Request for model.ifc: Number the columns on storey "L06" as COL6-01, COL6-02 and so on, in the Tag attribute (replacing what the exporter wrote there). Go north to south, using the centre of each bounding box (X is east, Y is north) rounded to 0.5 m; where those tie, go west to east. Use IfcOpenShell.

First a look at what the model holds.

```python
import ifcopenshell
import ifcopenshell.util.element
import ifcopenshell.util.placement

model = ifcopenshell.open("model.ifc")
print(model.schema)
storey = next(s for s in model.by_type("IfcBuildingStorey") if s.Name == "L06")
columns = [e for e in ifcopenshell.util.element.get_decomposition(storey) if e.is_a("IfcColumn")]
for e in sorted(columns, key=lambda e: e.id()):
    origin = ifcopenshell.util.placement.get_local_placement(e.ObjectPlacement)[:3, 3]
    print(e.id(), e.Tag, e.Name, origin.round(2) + 0.0, sep=" | ")
```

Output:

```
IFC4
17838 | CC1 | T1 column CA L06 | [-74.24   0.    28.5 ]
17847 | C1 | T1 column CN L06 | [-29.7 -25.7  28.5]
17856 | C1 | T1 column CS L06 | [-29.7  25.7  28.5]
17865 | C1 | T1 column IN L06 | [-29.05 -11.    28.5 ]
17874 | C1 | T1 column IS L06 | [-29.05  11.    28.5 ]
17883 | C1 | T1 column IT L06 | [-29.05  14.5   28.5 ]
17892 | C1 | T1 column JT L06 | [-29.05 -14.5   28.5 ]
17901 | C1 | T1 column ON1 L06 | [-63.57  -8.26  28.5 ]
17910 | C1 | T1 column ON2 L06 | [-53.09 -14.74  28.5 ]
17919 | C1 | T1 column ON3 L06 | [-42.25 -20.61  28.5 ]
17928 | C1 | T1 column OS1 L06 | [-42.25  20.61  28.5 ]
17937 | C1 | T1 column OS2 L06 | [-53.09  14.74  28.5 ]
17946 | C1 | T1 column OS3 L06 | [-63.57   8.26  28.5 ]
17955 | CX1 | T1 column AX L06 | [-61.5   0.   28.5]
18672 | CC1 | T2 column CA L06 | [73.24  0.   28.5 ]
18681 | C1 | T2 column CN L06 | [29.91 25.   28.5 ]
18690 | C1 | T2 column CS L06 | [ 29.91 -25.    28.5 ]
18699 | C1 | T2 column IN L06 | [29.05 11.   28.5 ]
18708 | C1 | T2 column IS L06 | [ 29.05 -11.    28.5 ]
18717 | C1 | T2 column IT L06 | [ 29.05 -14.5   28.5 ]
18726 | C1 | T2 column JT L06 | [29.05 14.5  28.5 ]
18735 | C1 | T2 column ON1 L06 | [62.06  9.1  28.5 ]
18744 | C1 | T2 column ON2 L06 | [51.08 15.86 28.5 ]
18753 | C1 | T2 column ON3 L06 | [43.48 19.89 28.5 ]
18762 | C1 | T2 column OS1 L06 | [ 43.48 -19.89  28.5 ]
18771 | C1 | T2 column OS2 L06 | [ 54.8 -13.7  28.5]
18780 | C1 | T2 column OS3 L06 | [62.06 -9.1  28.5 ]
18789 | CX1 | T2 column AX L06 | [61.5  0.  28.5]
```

```python
import ifcopenshell
import ifcopenshell.geom
import ifcopenshell.util.element
import ifcopenshell.util.shape

model = ifcopenshell.open("model.ifc")
settings = ifcopenshell.geom.settings()
settings.set("use-world-coords", True)


def centre(element):
    shape = ifcopenshell.geom.create_shape(settings, element)
    return ifcopenshell.util.shape.get_bbox_centroid(shape.geometry)


storey = next(s for s in model.by_type("IfcBuildingStorey") if s.Name == "L06")
columns = [e for e in ifcopenshell.util.element.get_decomposition(storey) if e.is_a("IfcColumn")]

# Insertion points can sit at a corner or the storey origin, so sort by the geometry (in metres).
centres = {e: centre(e) for e in columns}
columns.sort(key=lambda e: (-round(centres[e][1] / 0.5), centres[e][0]))

for i, e in enumerate(columns, start=1):
    number = f"COL6-{i:02d}"
    e.Tag = number
    print(e.id(), number)

model.write("model_v2.ifc")
```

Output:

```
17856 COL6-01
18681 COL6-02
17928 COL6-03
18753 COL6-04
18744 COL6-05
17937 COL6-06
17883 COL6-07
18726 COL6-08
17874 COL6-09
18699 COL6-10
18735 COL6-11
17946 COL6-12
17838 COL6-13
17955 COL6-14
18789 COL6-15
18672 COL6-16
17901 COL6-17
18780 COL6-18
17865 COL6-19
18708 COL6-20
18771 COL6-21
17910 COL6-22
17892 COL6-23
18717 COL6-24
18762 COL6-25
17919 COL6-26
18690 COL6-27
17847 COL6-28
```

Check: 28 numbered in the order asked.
